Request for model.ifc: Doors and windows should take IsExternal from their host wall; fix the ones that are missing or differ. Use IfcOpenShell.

First a look at what the model holds.

```python
import ifcopenshell
import ifcopenshell.util.element

model = ifcopenshell.open("model.ifc")
print(model.schema)
seen = {}
for e in model.by_type("IfcDoor") + model.by_type("IfcWindow"):
    if not e.FillsVoids:
        continue
    host = e.FillsVoids[0].RelatingOpeningElement.VoidsElements[0].RelatingBuildingElement
    own = ifcopenshell.util.element.get_pset(e, f"Pset_{e.is_a()[3:].removesuffix('StandardCase')}Common", "IsExternal")
    wall = ifcopenshell.util.element.get_pset(host, "Pset_WallCommon", "IsExternal")
    seen[e.is_a(), own, wall] = seen.get((e.is_a(), own, wall), 0) + 1
for (cls, own, wall), count in sorted(seen.items(), key=str):
    print(count, cls, "IsExternal:", own, "| host wall:", wall)
```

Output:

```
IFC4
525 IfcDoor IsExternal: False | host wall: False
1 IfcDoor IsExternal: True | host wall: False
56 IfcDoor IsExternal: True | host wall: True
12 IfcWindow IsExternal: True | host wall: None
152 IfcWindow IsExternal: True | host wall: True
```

```python
import ifcopenshell
import ifcopenshell.api.pset
import ifcopenshell.util.element

model = ifcopenshell.open("model.ifc")

count = 0
for ifc_class, pset_name in (("IfcDoor", "Pset_DoorCommon"), ("IfcWindow", "Pset_WindowCommon")):
    for e in model.by_type(ifc_class):
        if not e.FillsVoids:
            continue
        host = e.FillsVoids[0].RelatingOpeningElement.VoidsElements[0].RelatingBuildingElement
        external = ifcopenshell.util.element.get_pset(host, "Pset_WallCommon", "IsExternal")
        if external is None or ifcopenshell.util.element.get_pset(e, pset_name, "IsExternal") == external:
            continue
        pset = ifcopenshell.api.pset.add_pset(model, product=e, name=pset_name)
        ifcopenshell.api.pset.edit_pset(model, pset=pset, properties={"IsExternal": external})
        count += 1

print(count, "updated")

model.write("model_updated.ifc")
```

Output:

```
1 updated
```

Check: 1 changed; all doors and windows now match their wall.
